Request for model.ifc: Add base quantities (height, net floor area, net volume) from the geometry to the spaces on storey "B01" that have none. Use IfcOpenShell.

First a look at what the model holds.

```python
import ifcopenshell
import ifcopenshell.util.element
import ifcopenshell.util.unit

model = ifcopenshell.open("model.ifc")
print(model.schema)
for unit_type in ("LENGTHUNIT", "AREAUNIT", "VOLUMEUNIT"):
    print(unit_type, ifcopenshell.util.unit.calculate_unit_scale(model, unit_type))
storey = next(s for s in model.by_type("IfcBuildingStorey") if s.Name == "B01")
spaces = [e for e in ifcopenshell.util.element.get_decomposition(storey) if e.is_a("IfcSpace")]
for e in sorted(spaces, key=lambda e: e.id()):
    print(e.id(), e.is_a(), e.Name, list(ifcopenshell.util.element.get_psets(e, qtos_only=True)), sep=" | ")
```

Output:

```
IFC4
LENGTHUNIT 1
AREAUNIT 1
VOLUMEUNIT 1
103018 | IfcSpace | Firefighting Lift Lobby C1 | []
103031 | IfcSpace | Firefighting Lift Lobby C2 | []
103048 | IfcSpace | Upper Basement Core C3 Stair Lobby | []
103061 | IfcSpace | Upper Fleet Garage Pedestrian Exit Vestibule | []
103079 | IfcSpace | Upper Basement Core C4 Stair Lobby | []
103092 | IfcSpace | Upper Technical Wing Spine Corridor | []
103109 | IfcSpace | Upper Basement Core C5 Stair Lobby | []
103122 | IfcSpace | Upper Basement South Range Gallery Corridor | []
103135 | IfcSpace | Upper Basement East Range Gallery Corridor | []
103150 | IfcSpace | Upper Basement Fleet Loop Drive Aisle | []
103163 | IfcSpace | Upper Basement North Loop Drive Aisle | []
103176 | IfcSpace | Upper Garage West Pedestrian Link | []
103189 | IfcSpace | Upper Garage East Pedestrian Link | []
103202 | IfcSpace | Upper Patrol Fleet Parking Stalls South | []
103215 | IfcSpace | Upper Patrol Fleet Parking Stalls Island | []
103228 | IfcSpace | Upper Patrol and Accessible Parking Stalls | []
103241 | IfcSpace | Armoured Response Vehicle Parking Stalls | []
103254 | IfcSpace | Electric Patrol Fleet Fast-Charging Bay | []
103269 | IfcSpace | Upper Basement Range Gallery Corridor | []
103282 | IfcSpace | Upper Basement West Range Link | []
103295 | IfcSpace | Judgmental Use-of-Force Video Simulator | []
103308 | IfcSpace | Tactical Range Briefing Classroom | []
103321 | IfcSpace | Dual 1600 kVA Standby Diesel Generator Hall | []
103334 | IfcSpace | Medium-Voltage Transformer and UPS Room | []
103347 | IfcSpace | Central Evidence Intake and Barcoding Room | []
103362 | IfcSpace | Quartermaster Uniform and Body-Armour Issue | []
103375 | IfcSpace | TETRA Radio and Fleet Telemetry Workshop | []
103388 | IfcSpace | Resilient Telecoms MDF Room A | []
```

```python
import ifcopenshell
import ifcopenshell.api.pset
import ifcopenshell.geom
import ifcopenshell.util.element
import ifcopenshell.util.shape
import ifcopenshell.util.unit

model = ifcopenshell.open("model.ifc")
unit_scale = ifcopenshell.util.unit.calculate_unit_scale(model)
area_scale = ifcopenshell.util.unit.calculate_unit_scale(model, "AREAUNIT")
volume_scale = ifcopenshell.util.unit.calculate_unit_scale(model, "VOLUMEUNIT")
settings = ifcopenshell.geom.settings()

storey = next(s for s in model.by_type("IfcBuildingStorey") if s.Name == "B01")
spaces = [e for e in ifcopenshell.util.element.get_decomposition(storey) if e.is_a("IfcSpace")]

for e in sorted(spaces, key=lambda e: e.id()):
    if ifcopenshell.util.element.get_psets(e, qtos_only=True, should_inherit=False):
        continue
    # Geometry comes back in metres, in the element's own axes.
    shape = ifcopenshell.geom.create_shape(settings, e)
    values = {
        "Height": ifcopenshell.util.shape.get_z(shape.geometry) / unit_scale,
        "NetFloorArea": ifcopenshell.util.shape.get_footprint_area(shape.geometry) / area_scale,
        "NetVolume": ifcopenshell.util.shape.get_volume(shape.geometry) / volume_scale,
    }
    qto = ifcopenshell.api.pset.add_qto(model, product=e, name="Qto_SpaceBaseQuantities")
    ifcopenshell.api.pset.edit_qto(model, qto=qto, properties=values)
    print(e.id(), {k: round(v, 3) for k, v in values.items()})

model.write("model_v2.ifc")
```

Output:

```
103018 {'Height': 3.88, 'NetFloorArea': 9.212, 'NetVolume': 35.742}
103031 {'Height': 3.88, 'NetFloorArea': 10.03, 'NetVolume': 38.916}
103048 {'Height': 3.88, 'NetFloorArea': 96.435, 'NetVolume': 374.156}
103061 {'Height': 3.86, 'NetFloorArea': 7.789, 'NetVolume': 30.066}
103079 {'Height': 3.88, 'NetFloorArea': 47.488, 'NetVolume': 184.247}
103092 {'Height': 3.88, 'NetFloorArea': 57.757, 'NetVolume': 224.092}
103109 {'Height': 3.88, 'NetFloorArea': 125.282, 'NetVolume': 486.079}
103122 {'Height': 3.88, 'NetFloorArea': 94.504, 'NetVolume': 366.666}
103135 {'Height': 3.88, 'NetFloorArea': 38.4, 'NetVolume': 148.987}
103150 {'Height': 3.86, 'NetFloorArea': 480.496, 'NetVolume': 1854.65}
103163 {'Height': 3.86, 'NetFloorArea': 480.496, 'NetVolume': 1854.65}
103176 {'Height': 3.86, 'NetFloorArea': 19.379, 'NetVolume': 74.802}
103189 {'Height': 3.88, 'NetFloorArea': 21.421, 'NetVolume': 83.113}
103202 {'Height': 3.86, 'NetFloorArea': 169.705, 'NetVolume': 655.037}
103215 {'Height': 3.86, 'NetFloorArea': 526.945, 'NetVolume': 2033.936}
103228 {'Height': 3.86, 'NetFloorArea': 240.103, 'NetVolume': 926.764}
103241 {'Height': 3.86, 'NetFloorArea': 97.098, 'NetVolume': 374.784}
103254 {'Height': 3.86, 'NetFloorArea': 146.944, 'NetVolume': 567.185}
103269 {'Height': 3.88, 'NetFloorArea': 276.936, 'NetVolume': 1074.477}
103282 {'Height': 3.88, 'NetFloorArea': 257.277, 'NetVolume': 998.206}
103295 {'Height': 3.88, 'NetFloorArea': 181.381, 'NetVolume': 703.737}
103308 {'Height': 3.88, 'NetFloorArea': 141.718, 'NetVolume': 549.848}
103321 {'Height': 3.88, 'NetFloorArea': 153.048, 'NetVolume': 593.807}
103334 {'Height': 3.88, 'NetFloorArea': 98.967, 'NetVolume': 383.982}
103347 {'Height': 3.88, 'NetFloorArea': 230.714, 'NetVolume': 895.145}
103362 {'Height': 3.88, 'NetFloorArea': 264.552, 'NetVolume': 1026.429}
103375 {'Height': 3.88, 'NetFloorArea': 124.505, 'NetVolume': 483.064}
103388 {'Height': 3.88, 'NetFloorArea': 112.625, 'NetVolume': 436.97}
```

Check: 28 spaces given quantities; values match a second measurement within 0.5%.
